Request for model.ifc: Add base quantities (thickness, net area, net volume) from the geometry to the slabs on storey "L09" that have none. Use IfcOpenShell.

First a look at what the model holds.

```python
import ifcopenshell
import ifcopenshell.util.element
import ifcopenshell.util.unit

model = ifcopenshell.open("model.ifc")
print(model.schema)
for unit_type in ("LENGTHUNIT", "AREAUNIT", "VOLUMEUNIT"):
    print(unit_type, ifcopenshell.util.unit.calculate_unit_scale(model, unit_type))
storey = next(s for s in model.by_type("IfcBuildingStorey") if s.Name == "L09")
slabs = [e for e in ifcopenshell.util.element.get_decomposition(storey) if e.is_a("IfcSlab")]
for e in sorted(slabs, key=lambda e: e.id()):
    print(e.id(), e.is_a(), e.Name, list(ifcopenshell.util.element.get_psets(e, qtos_only=True)), sep=" | ")
```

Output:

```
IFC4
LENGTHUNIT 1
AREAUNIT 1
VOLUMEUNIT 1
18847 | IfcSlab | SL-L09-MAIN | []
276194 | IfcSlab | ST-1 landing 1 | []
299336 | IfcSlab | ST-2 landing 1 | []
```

```python
import ifcopenshell
import ifcopenshell.api.pset
import ifcopenshell.geom
import ifcopenshell.util.element
import ifcopenshell.util.shape
import ifcopenshell.util.unit

model = ifcopenshell.open("model.ifc")
unit_scale = ifcopenshell.util.unit.calculate_unit_scale(model)
area_scale = ifcopenshell.util.unit.calculate_unit_scale(model, "AREAUNIT")
volume_scale = ifcopenshell.util.unit.calculate_unit_scale(model, "VOLUMEUNIT")
settings = ifcopenshell.geom.settings()

storey = next(s for s in model.by_type("IfcBuildingStorey") if s.Name == "L09")
slabs = [e for e in ifcopenshell.util.element.get_decomposition(storey) if e.is_a("IfcSlab")]

for e in sorted(slabs, key=lambda e: e.id()):
    if ifcopenshell.util.element.get_psets(e, qtos_only=True, should_inherit=False):
        continue
    # Geometry comes back in metres, in the element's own axes.
    shape = ifcopenshell.geom.create_shape(settings, e)
    values = {
        "Width": ifcopenshell.util.shape.get_z(shape.geometry) / unit_scale,
        "NetArea": ifcopenshell.util.shape.get_footprint_area(shape.geometry) / area_scale,
        "NetVolume": ifcopenshell.util.shape.get_volume(shape.geometry) / volume_scale,
    }
    qto = ifcopenshell.api.pset.add_qto(model, product=e, name="Qto_SlabBaseQuantities")
    ifcopenshell.api.pset.edit_qto(model, qto=qto, properties=values)
    print(e.id(), {k: round(v, 3) for k, v in values.items()})

model.write("model_v2.ifc")
```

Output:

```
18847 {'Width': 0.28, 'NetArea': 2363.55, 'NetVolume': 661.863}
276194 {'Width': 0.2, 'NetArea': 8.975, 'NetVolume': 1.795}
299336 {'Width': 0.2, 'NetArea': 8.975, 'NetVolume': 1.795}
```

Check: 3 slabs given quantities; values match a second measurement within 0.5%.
